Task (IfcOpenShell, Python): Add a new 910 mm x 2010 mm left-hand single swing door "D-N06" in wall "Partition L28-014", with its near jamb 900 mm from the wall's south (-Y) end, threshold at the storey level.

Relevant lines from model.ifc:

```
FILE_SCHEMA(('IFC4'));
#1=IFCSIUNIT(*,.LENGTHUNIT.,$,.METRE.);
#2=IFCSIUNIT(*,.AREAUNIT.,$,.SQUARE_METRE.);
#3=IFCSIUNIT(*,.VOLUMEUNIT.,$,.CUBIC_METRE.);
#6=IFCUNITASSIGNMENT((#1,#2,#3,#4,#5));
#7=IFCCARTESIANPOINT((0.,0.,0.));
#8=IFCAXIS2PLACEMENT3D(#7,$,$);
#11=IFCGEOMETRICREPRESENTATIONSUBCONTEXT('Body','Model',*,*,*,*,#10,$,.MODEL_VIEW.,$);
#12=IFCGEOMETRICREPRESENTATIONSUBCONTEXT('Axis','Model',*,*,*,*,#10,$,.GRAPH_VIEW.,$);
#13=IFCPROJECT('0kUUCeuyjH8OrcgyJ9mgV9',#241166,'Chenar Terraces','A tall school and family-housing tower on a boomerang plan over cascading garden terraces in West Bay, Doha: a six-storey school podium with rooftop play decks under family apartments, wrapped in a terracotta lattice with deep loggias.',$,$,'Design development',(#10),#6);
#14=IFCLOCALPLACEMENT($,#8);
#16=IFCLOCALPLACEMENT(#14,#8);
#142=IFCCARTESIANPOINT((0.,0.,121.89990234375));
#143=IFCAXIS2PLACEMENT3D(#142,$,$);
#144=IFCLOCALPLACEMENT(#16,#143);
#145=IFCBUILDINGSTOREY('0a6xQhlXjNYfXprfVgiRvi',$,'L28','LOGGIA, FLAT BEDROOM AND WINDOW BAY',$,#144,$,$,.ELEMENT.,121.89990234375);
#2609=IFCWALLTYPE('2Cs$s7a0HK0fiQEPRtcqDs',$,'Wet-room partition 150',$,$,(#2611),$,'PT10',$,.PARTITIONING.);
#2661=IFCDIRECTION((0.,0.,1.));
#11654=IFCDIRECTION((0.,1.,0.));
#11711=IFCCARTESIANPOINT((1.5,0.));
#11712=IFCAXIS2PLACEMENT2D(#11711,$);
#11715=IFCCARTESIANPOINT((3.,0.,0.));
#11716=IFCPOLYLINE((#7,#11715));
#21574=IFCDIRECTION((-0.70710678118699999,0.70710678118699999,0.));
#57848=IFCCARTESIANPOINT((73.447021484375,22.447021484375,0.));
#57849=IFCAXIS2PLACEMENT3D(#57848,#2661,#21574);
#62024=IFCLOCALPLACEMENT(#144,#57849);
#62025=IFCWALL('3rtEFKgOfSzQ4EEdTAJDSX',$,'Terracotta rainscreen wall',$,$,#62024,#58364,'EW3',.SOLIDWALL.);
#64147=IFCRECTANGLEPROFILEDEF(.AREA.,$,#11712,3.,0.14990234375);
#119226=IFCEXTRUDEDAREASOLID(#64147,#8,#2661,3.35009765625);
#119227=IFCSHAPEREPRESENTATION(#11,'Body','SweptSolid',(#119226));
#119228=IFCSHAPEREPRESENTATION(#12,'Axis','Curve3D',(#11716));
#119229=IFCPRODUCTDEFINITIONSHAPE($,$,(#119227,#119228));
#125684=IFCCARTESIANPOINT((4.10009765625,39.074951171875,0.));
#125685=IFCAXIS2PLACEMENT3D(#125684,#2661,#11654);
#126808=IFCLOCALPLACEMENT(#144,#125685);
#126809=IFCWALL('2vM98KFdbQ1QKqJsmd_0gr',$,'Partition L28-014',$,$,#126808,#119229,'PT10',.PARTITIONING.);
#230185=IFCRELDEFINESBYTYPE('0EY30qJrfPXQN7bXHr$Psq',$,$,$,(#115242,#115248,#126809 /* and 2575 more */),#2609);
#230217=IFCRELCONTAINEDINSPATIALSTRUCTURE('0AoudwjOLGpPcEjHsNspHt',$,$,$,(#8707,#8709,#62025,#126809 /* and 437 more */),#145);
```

```python
import numpy as np
import ifcopenshell
import ifcopenshell.api.feature
import ifcopenshell.api.geometry
import ifcopenshell.api.root
import ifcopenshell.api.spatial
import ifcopenshell.geom
import ifcopenshell.util.element
import ifcopenshell.util.placement
import ifcopenshell.util.representation
import ifcopenshell.util.shape
import ifcopenshell.util.unit

model = ifcopenshell.open("model.ifc")
unit_scale = ifcopenshell.util.unit.calculate_unit_scale(model)
settings = ifcopenshell.geom.settings()


def volume(element):
    """Net volume in cubic metres, openings subtracted."""
    shape = ifcopenshell.geom.create_shape(settings, element)
    return ifcopenshell.util.shape.get_volume(shape.geometry)


wall = model.by_guid("2vM98KFdbQ1QKqJsmd_0gr")
storey = ifcopenshell.util.element.get_container(wall, ifc_class="IfcBuildingStorey")
context = ifcopenshell.util.representation.get_context(model, "Model", "Body", "MODEL_VIEW")
before = volume(wall)

width, height, from_end, sill = 0.91, 2.01, 0.9, 0.0  # metres

# The wall runs along its own X axis, and the end named is its -X end.
wall_shape = ifcopenshell.geom.create_shape(settings, wall)
x, y, z = ifcopenshell.util.shape.get_vertices(wall_shape.geometry).T
start = x.min() + from_end
face, thickness = float(y.min()), float(y.max() - y.min())
wall_matrix = ifcopenshell.util.placement.get_local_placement(wall.ObjectPlacement)
level = ifcopenshell.util.placement.get_local_placement(storey.ObjectPlacement)[2, 3]


def in_wall(x, y):
    """Placement at x, y metres in the wall's axes, at sill height."""
    matrix = wall_matrix.copy()
    matrix[:, 3] = wall_matrix @ np.array([x / unit_scale, y / unit_scale, 0.0, 1.0])
    matrix[2, 3] = level + sill / unit_scale
    return matrix


# Opening: a box that overshoots both wall faces by 50 mm.
opening = ifcopenshell.api.root.create_entity(model, ifc_class="IfcOpeningElement", predefined_type="OPENING")
box = ifcopenshell.api.geometry.add_wall_representation(
    model, context=context, length=width, height=height, thickness=thickness + 0.1
)
ifcopenshell.api.geometry.assign_representation(model, product=opening, representation=box)
ifcopenshell.api.geometry.edit_object_placement(model, product=opening, matrix=in_wall(start, face - 0.05), is_si=False)
ifcopenshell.api.feature.add_feature(model, feature=opening, element=wall)

door = ifcopenshell.api.root.create_entity(model, ifc_class="IfcDoor", name="D-N06", predefined_type="DOOR")
door.OverallWidth, door.OverallHeight = width / unit_scale, height / unit_scale
door.OperationType = "SINGLE_SWING_LEFT"
body = ifcopenshell.api.geometry.add_door_representation(
    model,
    context=context,
    overall_width=door.OverallWidth,
    overall_height=door.OverallHeight,
    operation_type="SINGLE_SWING_LEFT",
    lining_properties={"LiningDepth": thickness / unit_scale, "ThresholdDepth": thickness / unit_scale},
)
ifcopenshell.api.geometry.assign_representation(model, product=door, representation=body)
ifcopenshell.api.spatial.assign_container(model, products=[door], relating_structure=storey)
ifcopenshell.api.feature.add_filling(model, opening=opening, element=door)

# The lining spans the wall, so the door starts at the wall face.
ifcopenshell.api.geometry.edit_object_placement(model, product=door, matrix=in_wall(start, face), is_si=False)

after = volume(wall)

print(f"wall volume {before:.3f} -> {after:.3f} m3")

model.write("model-out.ifc")
```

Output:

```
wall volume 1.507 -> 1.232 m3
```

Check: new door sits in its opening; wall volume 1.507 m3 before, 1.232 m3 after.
